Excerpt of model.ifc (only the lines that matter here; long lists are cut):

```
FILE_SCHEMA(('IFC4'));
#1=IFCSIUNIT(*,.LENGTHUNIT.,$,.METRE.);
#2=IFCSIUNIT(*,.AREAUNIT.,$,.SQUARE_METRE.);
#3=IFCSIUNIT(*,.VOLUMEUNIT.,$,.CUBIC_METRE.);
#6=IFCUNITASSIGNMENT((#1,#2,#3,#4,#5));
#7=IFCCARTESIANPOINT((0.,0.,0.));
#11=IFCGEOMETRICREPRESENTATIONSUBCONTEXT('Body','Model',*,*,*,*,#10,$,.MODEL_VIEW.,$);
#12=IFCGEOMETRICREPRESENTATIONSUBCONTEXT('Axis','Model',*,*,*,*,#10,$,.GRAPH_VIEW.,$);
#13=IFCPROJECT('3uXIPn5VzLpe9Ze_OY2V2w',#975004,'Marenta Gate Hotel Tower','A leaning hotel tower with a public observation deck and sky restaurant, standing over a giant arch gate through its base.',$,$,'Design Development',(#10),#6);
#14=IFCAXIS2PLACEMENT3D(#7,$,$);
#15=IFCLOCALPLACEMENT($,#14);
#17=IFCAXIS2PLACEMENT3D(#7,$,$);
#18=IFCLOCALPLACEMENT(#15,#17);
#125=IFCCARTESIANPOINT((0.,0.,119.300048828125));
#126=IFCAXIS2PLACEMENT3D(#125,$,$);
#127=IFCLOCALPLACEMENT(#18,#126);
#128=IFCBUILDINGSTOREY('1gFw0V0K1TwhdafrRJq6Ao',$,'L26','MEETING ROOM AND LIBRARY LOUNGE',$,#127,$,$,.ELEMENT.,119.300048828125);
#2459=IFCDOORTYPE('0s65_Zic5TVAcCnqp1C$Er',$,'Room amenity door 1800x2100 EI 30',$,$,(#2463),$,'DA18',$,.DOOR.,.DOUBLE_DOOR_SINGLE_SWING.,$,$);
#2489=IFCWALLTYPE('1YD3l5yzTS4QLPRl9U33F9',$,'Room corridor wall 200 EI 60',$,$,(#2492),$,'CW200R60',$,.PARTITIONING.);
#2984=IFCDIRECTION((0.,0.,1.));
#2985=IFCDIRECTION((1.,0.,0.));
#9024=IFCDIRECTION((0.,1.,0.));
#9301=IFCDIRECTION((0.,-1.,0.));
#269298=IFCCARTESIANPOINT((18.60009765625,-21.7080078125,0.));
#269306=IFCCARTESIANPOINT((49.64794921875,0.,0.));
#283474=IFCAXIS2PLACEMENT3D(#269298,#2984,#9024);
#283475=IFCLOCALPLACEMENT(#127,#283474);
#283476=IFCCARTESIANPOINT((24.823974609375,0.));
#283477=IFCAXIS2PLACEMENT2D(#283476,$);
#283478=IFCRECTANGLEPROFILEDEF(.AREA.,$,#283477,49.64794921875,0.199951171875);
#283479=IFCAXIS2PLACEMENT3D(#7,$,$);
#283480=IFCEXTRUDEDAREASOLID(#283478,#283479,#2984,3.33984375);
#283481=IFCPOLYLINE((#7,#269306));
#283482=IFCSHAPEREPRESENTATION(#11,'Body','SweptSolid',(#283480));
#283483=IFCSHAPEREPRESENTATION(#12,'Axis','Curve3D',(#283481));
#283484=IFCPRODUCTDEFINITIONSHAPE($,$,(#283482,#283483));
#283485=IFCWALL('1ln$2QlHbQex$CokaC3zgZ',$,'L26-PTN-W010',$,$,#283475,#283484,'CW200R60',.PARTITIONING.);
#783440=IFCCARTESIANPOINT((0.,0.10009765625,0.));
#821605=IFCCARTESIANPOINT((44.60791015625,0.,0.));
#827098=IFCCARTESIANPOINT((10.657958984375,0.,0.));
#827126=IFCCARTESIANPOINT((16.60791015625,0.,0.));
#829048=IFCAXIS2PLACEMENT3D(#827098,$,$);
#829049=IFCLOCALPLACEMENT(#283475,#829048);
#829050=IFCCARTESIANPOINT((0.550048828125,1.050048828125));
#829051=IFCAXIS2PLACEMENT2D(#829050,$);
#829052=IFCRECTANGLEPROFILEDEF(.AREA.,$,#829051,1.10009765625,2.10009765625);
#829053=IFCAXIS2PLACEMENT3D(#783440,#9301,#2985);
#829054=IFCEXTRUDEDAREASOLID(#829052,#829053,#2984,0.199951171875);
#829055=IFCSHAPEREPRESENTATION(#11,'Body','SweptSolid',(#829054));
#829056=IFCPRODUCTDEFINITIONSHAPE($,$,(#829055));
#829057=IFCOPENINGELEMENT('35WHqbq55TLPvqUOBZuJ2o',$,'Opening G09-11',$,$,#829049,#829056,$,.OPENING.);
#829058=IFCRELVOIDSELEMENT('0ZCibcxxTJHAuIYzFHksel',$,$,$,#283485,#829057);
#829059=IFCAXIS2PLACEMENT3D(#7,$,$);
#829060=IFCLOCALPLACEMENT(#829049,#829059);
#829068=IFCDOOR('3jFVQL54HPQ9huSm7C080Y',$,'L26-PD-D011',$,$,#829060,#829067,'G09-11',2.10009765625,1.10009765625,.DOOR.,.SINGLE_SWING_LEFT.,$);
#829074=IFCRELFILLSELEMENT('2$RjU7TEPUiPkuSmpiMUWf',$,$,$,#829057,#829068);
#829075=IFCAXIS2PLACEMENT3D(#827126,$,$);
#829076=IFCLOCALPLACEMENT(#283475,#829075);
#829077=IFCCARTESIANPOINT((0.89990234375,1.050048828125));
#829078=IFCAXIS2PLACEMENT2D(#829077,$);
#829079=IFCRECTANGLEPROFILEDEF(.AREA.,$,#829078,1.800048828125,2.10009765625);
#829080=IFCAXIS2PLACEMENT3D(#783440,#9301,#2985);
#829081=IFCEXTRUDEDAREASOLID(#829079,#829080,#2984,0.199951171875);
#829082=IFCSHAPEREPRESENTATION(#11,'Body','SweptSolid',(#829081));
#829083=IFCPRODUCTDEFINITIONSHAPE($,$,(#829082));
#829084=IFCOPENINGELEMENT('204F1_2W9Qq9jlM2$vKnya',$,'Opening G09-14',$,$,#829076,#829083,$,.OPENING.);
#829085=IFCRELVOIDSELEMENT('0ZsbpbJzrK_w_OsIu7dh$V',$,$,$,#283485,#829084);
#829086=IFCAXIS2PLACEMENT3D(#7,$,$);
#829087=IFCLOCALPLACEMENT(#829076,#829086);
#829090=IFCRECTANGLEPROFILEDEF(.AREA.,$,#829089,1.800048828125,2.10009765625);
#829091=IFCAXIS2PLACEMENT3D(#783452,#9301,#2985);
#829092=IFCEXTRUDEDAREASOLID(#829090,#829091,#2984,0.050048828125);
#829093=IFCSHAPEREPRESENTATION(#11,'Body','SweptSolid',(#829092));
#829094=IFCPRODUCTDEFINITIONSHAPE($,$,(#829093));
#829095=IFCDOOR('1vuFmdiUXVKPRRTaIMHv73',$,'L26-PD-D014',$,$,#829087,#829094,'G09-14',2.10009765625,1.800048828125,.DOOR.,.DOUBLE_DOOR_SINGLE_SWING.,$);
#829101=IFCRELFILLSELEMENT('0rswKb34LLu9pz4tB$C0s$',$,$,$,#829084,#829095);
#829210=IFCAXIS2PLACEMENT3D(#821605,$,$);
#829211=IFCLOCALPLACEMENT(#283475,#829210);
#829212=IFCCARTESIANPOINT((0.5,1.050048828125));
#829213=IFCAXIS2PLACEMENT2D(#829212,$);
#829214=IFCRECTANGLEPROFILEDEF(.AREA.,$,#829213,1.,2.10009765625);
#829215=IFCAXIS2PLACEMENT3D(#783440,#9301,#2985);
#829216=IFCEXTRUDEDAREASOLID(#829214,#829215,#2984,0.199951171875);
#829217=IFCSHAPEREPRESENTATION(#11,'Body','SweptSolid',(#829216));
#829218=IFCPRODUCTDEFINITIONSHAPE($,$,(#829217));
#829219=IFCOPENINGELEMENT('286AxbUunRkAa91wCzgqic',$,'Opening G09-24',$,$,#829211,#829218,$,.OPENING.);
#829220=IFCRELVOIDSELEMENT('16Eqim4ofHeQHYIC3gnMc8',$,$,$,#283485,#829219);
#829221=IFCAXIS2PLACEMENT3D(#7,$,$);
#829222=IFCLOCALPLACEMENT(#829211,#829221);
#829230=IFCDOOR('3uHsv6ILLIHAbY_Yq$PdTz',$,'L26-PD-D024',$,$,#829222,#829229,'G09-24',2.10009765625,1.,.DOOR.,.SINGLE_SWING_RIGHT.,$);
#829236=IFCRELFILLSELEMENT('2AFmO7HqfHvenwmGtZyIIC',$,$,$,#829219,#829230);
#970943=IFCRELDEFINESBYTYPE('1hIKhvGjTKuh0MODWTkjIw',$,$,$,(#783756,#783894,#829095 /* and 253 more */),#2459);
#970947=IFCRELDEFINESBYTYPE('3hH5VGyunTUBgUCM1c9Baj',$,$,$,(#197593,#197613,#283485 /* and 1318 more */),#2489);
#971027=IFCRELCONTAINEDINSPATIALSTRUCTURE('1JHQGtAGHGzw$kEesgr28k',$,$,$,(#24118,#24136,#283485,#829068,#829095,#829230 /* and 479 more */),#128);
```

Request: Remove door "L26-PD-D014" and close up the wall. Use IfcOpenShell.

```python
import ifcopenshell
import ifcopenshell.api.feature
import ifcopenshell.api.root
import ifcopenshell.geom
import ifcopenshell.util.shape

model = ifcopenshell.open("model.ifc")
settings = ifcopenshell.geom.settings()


def volume(element):
    """Net volume in cubic metres, openings subtracted."""
    shape = ifcopenshell.geom.create_shape(settings, element)
    return ifcopenshell.util.shape.get_volume(shape.geometry)


door = model.by_guid("1vuFmdiUXVKPRRTaIMHv73")
opening = door.FillsVoids[0].RelatingOpeningElement
wall = opening.VoidsElements[0].RelatingBuildingElement
before = volume(wall)

ifcopenshell.api.root.remove_product(model, product=door)
ifcopenshell.api.feature.remove_feature(model, feature=opening)

after = volume(wall)

print(f"wall volume {before:.3f} -> {after:.3f} m3")

model.write("model_v2.ifc")
```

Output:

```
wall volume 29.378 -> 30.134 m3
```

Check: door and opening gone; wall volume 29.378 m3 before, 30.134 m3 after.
